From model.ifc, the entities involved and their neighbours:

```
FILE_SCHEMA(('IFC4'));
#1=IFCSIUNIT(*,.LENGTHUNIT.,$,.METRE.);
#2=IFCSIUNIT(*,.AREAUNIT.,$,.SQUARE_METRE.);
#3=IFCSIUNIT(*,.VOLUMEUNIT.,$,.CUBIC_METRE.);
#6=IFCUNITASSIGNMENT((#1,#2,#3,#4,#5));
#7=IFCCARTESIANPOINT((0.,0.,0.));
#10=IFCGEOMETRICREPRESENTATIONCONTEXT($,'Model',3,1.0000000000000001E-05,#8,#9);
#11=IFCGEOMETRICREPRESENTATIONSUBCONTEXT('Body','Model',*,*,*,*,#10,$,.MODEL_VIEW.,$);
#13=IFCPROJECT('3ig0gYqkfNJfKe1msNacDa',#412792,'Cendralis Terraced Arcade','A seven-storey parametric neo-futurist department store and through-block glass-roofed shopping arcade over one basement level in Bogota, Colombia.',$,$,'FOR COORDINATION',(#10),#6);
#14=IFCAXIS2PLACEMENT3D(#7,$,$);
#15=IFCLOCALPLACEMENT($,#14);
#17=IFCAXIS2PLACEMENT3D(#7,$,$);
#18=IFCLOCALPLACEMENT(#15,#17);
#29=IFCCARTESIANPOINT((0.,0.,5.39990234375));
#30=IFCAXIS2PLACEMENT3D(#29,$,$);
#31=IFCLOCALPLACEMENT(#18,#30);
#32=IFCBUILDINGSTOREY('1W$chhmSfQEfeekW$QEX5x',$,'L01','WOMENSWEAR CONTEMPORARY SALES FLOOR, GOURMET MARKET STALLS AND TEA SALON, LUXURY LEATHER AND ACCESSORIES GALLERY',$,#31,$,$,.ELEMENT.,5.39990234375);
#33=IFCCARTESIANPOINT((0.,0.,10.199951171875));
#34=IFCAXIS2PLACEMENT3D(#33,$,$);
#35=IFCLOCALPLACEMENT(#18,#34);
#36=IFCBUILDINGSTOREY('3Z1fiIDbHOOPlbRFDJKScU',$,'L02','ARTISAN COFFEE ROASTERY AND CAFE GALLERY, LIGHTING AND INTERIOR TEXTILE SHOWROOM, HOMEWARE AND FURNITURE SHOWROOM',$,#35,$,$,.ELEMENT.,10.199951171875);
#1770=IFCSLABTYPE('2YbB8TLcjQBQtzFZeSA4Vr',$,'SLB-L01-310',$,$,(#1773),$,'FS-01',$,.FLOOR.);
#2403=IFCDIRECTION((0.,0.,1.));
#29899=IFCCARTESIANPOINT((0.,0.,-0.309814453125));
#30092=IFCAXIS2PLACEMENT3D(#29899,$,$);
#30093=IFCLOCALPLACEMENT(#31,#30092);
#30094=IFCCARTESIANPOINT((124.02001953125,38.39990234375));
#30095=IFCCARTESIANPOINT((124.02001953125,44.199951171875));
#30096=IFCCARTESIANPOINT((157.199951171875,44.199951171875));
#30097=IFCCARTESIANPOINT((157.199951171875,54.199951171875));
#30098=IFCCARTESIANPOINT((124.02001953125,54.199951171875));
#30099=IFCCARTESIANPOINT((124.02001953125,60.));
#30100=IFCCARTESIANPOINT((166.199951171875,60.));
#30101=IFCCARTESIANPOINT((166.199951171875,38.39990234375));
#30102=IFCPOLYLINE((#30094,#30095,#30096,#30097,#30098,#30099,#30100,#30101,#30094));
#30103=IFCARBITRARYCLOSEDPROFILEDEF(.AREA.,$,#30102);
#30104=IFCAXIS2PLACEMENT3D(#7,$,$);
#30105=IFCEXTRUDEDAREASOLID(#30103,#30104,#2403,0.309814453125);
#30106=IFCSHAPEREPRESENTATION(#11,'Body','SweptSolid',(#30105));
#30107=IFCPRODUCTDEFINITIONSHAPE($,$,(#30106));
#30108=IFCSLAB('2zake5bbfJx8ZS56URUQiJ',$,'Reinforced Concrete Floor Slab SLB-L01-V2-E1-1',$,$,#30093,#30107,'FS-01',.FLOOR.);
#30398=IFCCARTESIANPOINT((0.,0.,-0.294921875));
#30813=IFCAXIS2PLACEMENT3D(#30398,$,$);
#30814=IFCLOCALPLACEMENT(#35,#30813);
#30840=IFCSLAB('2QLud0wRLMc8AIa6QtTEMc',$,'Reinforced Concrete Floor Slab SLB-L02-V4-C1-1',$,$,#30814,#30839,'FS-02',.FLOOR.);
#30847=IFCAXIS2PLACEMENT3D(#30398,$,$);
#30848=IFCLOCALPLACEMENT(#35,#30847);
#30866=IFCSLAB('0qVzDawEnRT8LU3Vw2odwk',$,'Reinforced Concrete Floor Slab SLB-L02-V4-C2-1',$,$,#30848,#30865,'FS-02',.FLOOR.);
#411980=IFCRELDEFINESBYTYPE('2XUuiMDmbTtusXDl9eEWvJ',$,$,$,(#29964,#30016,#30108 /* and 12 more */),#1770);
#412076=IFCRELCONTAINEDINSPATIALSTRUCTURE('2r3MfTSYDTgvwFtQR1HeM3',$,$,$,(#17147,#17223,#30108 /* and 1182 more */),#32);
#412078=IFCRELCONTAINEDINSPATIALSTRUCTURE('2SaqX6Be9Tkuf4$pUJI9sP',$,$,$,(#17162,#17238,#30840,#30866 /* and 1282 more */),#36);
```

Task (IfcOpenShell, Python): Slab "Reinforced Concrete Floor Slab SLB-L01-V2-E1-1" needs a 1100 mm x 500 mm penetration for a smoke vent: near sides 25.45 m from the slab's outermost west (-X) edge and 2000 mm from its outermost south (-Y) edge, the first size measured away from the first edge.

```python
import numpy as np
import ifcopenshell
import ifcopenshell.api.feature
import ifcopenshell.api.geometry
import ifcopenshell.api.root
import ifcopenshell.geom
import ifcopenshell.util.placement
import ifcopenshell.util.representation
import ifcopenshell.util.shape
import ifcopenshell.util.unit

model = ifcopenshell.open("model.ifc")
unit_scale = ifcopenshell.util.unit.calculate_unit_scale(model)
settings = ifcopenshell.geom.settings()


def volume(element):
    """Net volume in cubic metres, openings subtracted."""
    shape = ifcopenshell.geom.create_shape(settings, element)
    return ifcopenshell.util.shape.get_volume(shape.geometry)


slab = model.by_guid("2zake5bbfJx8ZS56URUQiJ")
before = volume(slab)

# Extent in the slab's own axes, in metres. The edges named are its -X and -Y sides.
slab_shape = ifcopenshell.geom.create_shape(settings, slab)
vertices = ifcopenshell.util.shape.get_vertices(slab_shape.geometry)
x_min, y_min, bottom = vertices.min(axis=0)
top = vertices[:, 2].max()

opening = ifcopenshell.api.root.create_entity(model, ifc_class="IfcOpeningElement", name="Smoke vent opening", predefined_type="OPENING")
context = ifcopenshell.util.representation.get_context(model, "Model", "Body", "MODEL_VIEW")
width, depth = 1.1, 0.5
outline = [(0.0, 0.0), (width, 0.0), (width, depth), (0.0, depth), (0.0, 0.0)]
# Overshoot both faces by 50 mm so the cut is clean.
shape = ifcopenshell.api.geometry.add_slab_representation(
    model, context=context, depth=top - bottom + 0.1, polyline=outline
)
ifcopenshell.api.geometry.assign_representation(model, product=opening, representation=shape)

matrix = ifcopenshell.util.placement.get_local_placement(slab.ObjectPlacement)
matrix[:, 3] = matrix @ np.append(np.array([x_min + 25.45, y_min + 2, bottom - 0.05]) / unit_scale, 1.0)
ifcopenshell.api.geometry.edit_object_placement(model, product=opening, matrix=matrix, is_si=False)
ifcopenshell.api.feature.add_feature(model, feature=opening, element=slab)

after = volume(slab)

print(f"slab volume {before:.3f} -> {after:.3f} m3")

model.write("model_rev.ifc")
```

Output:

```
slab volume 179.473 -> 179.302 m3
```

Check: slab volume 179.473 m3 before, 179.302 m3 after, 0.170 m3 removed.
